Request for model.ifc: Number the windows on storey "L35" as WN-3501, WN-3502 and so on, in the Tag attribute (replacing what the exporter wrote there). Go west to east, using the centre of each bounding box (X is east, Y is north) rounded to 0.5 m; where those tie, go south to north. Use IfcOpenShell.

First a look at what the model holds.

```python
import ifcopenshell
import ifcopenshell.util.element
import ifcopenshell.util.placement

model = ifcopenshell.open("model.ifc")
print(model.schema)
storey = next(s for s in model.by_type("IfcBuildingStorey") if s.Name == "L35")
windows = [e for e in ifcopenshell.util.element.get_decomposition(storey) if e.is_a("IfcWindow")]
for e in sorted(windows, key=lambda e: e.id()):
    origin = ifcopenshell.util.placement.get_local_placement(e.ObjectPlacement)[:3, 3]
    print(e.id(), e.Tag, e.Name, origin.round(2) + 0.0, sep=" | ")
```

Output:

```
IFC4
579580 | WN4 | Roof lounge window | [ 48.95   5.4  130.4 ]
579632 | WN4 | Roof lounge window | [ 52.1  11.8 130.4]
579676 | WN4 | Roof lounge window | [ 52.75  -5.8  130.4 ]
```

```python
import ifcopenshell
import ifcopenshell.geom
import ifcopenshell.util.element
import ifcopenshell.util.shape

model = ifcopenshell.open("model.ifc")
settings = ifcopenshell.geom.settings()
settings.set("use-world-coords", True)


def centre(element):
    shape = ifcopenshell.geom.create_shape(settings, element)
    return ifcopenshell.util.shape.get_bbox_centroid(shape.geometry)


storey = next(s for s in model.by_type("IfcBuildingStorey") if s.Name == "L35")
windows = [e for e in ifcopenshell.util.element.get_decomposition(storey) if e.is_a("IfcWindow")]

# Insertion points can sit at a corner or the storey origin, so sort by the geometry (in metres).
centres = {e: centre(e) for e in windows}
windows.sort(key=lambda e: (round(centres[e][0] / 0.5), centres[e][1]))

for i, e in enumerate(windows, start=1):
    number = f"WN-35{i:02d}"
    e.Tag = number
    print(e.id(), number)

model.write("model_rev.ifc")
```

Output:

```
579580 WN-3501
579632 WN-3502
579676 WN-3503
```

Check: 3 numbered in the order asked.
